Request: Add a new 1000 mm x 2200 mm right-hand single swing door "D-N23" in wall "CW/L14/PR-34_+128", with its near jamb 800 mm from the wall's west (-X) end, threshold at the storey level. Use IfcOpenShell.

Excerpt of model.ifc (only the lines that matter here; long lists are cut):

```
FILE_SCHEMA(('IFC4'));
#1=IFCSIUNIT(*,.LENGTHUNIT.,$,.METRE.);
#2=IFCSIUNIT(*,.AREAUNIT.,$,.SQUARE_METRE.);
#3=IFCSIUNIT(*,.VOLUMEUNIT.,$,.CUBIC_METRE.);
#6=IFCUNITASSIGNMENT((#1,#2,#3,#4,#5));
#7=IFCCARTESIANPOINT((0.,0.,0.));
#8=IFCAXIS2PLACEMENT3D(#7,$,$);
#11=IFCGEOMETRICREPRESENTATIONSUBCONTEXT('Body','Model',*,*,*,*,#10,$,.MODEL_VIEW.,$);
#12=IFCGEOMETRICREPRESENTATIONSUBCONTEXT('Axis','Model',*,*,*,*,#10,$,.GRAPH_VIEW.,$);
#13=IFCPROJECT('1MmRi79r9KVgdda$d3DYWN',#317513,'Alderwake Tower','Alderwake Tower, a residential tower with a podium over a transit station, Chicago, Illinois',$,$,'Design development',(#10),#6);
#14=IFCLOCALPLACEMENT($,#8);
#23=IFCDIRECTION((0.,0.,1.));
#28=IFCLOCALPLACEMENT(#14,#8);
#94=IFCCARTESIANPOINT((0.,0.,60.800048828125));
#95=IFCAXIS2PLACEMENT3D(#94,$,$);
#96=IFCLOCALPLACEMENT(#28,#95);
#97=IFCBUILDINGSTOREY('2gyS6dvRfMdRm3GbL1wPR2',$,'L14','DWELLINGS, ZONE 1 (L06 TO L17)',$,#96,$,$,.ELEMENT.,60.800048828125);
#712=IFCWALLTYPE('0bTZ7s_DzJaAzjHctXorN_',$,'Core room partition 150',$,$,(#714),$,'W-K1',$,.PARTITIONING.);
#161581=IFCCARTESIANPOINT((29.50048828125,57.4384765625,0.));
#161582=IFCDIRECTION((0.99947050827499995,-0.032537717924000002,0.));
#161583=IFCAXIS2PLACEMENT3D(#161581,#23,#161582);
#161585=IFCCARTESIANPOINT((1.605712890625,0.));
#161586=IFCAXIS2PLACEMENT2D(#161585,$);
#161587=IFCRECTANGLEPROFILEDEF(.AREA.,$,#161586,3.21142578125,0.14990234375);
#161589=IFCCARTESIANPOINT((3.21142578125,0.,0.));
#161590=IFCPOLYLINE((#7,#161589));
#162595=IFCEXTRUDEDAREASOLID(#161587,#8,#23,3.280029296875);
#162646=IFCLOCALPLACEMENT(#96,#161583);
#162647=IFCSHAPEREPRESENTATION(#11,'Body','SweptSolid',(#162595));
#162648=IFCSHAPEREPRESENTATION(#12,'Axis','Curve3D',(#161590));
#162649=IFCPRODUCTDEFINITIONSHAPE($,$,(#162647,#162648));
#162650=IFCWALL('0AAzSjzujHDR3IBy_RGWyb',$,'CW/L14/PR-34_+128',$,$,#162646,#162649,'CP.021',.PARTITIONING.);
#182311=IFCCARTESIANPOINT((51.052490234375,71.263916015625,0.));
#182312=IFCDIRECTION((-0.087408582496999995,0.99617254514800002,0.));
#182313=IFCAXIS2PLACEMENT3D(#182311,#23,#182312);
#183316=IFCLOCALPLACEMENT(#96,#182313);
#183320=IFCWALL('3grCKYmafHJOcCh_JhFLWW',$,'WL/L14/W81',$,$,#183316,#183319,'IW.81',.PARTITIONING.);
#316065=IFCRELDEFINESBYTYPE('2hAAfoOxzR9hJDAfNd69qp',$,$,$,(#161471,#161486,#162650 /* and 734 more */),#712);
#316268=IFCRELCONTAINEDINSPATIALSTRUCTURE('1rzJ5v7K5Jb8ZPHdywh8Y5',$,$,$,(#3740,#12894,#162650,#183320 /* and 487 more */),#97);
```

```python
import numpy as np
import ifcopenshell
import ifcopenshell.api.feature
import ifcopenshell.api.geometry
import ifcopenshell.api.root
import ifcopenshell.api.spatial
import ifcopenshell.geom
import ifcopenshell.util.element
import ifcopenshell.util.placement
import ifcopenshell.util.representation
import ifcopenshell.util.shape
import ifcopenshell.util.unit

model = ifcopenshell.open("model.ifc")
unit_scale = ifcopenshell.util.unit.calculate_unit_scale(model)
settings = ifcopenshell.geom.settings()


def volume(element):
    """Net volume in cubic metres, openings subtracted."""
    shape = ifcopenshell.geom.create_shape(settings, element)
    return ifcopenshell.util.shape.get_volume(shape.geometry)


wall = model.by_guid("0AAzSjzujHDR3IBy_RGWyb")
storey = ifcopenshell.util.element.get_container(wall, ifc_class="IfcBuildingStorey")
context = ifcopenshell.util.representation.get_context(model, "Model", "Body", "MODEL_VIEW")
before = volume(wall)

width, height, from_end, sill = 1, 2.2, 0.8, 0.0  # metres

# The wall runs along its own X axis, and the end named is its -X end.
wall_shape = ifcopenshell.geom.create_shape(settings, wall)
x, y, z = ifcopenshell.util.shape.get_vertices(wall_shape.geometry).T
start = x.min() + from_end
face, thickness = float(y.min()), float(y.max() - y.min())
wall_matrix = ifcopenshell.util.placement.get_local_placement(wall.ObjectPlacement)
level = ifcopenshell.util.placement.get_local_placement(storey.ObjectPlacement)[2, 3]


def in_wall(x, y):
    """Placement at x, y metres in the wall's axes, at sill height."""
    matrix = wall_matrix.copy()
    matrix[:, 3] = wall_matrix @ np.array([x / unit_scale, y / unit_scale, 0.0, 1.0])
    matrix[2, 3] = level + sill / unit_scale
    return matrix


# Opening: a box that overshoots both wall faces by 50 mm.
opening = ifcopenshell.api.root.create_entity(model, ifc_class="IfcOpeningElement", predefined_type="OPENING")
box = ifcopenshell.api.geometry.add_wall_representation(
    model, context=context, length=width, height=height, thickness=thickness + 0.1
)
ifcopenshell.api.geometry.assign_representation(model, product=opening, representation=box)
ifcopenshell.api.geometry.edit_object_placement(model, product=opening, matrix=in_wall(start, face - 0.05), is_si=False)
ifcopenshell.api.feature.add_feature(model, feature=opening, element=wall)

door = ifcopenshell.api.root.create_entity(model, ifc_class="IfcDoor", name="D-N23", predefined_type="DOOR")
door.OverallWidth, door.OverallHeight = width / unit_scale, height / unit_scale
door.OperationType = "SINGLE_SWING_RIGHT"
body = ifcopenshell.api.geometry.add_door_representation(
    model,
    context=context,
    overall_width=door.OverallWidth,
    overall_height=door.OverallHeight,
    operation_type="SINGLE_SWING_RIGHT",
    lining_properties={"LiningDepth": thickness / unit_scale, "ThresholdDepth": thickness / unit_scale},
)
ifcopenshell.api.geometry.assign_representation(model, product=door, representation=body)
ifcopenshell.api.spatial.assign_container(model, products=[door], relating_structure=storey)
ifcopenshell.api.feature.add_filling(model, opening=opening, element=door)

# The lining spans the wall, so the door starts at the wall face.
ifcopenshell.api.geometry.edit_object_placement(model, product=door, matrix=in_wall(start, face), is_si=False)

after = volume(wall)

print(f"wall volume {before:.3f} -> {after:.3f} m3")

model.write("model_rev.ifc")
```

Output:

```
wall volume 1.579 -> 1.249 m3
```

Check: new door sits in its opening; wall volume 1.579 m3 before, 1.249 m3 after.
